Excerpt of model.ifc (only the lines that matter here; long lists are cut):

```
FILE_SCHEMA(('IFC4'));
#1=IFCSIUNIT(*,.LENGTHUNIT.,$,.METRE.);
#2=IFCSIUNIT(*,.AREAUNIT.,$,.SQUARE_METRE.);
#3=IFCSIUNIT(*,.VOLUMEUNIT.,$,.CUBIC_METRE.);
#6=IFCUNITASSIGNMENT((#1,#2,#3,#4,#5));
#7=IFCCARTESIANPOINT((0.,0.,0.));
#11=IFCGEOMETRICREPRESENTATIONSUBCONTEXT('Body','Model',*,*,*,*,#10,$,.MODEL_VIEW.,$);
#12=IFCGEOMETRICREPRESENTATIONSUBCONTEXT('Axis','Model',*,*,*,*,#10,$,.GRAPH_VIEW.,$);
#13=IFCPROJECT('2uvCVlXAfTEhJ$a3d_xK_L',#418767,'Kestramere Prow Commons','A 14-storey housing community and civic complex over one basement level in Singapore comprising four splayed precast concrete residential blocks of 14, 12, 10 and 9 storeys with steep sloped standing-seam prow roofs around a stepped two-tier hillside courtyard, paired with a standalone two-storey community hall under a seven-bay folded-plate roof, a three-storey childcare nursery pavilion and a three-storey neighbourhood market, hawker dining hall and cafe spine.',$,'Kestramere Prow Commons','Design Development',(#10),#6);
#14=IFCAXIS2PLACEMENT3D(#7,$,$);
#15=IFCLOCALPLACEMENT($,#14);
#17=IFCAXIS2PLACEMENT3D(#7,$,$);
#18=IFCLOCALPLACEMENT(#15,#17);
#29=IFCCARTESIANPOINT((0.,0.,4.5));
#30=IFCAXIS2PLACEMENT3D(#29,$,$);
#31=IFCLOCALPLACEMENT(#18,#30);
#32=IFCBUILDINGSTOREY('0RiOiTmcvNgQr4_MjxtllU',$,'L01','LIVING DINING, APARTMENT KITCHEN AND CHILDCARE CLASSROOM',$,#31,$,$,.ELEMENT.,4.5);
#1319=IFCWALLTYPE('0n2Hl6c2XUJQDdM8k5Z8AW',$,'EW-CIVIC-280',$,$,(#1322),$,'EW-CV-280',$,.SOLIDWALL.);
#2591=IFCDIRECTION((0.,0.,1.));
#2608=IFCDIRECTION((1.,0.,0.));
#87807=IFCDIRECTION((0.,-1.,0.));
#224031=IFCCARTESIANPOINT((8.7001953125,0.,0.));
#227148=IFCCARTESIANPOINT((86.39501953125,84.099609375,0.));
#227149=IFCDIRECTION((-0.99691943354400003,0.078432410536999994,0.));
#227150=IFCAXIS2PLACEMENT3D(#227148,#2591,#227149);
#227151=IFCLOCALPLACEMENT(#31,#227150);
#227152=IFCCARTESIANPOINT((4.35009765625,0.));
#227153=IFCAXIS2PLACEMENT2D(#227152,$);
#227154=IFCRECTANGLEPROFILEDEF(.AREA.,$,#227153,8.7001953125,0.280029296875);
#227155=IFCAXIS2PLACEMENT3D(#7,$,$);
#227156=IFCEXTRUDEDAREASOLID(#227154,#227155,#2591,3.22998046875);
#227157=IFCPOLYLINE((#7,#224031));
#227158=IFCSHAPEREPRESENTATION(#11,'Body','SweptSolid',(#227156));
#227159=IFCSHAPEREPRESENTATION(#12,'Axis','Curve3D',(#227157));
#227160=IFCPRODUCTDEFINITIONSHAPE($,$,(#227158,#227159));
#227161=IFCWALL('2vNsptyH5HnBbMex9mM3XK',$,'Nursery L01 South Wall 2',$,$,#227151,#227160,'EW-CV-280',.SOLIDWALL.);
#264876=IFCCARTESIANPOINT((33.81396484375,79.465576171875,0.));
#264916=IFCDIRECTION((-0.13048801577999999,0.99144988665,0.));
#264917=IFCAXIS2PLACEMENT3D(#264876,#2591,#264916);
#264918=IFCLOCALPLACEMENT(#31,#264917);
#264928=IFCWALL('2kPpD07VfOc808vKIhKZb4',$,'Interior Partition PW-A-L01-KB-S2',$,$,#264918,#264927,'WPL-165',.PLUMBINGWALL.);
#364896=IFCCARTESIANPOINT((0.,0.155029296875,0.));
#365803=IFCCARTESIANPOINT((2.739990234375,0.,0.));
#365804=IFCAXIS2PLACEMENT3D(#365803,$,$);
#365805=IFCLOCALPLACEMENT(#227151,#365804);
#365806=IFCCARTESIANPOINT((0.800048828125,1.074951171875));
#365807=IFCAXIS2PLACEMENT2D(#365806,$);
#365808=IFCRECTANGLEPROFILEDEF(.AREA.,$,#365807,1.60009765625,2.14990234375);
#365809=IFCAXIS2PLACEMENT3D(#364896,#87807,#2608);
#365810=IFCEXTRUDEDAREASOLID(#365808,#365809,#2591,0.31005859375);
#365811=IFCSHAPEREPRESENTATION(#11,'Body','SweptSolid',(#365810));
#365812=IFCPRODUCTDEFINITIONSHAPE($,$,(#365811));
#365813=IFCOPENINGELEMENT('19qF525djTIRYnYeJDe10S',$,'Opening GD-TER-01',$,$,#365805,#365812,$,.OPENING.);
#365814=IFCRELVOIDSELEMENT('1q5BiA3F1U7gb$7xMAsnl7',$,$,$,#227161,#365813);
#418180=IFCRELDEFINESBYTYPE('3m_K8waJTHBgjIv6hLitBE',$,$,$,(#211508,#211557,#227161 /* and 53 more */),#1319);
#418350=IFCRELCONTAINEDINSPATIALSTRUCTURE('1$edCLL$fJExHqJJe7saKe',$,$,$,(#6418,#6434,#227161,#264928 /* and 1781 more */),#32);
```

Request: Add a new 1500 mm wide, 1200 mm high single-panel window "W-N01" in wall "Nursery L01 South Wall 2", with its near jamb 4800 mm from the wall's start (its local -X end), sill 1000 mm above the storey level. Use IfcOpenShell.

```python
import numpy as np
import ifcopenshell
import ifcopenshell.api.feature
import ifcopenshell.api.geometry
import ifcopenshell.api.root
import ifcopenshell.api.spatial
import ifcopenshell.geom
import ifcopenshell.util.element
import ifcopenshell.util.placement
import ifcopenshell.util.representation
import ifcopenshell.util.shape
import ifcopenshell.util.unit

model = ifcopenshell.open("model.ifc")
unit_scale = ifcopenshell.util.unit.calculate_unit_scale(model)
settings = ifcopenshell.geom.settings()


def volume(element):
    """Net volume in cubic metres, openings subtracted."""
    shape = ifcopenshell.geom.create_shape(settings, element)
    return ifcopenshell.util.shape.get_volume(shape.geometry)


wall = model.by_id(227161)
storey = ifcopenshell.util.element.get_container(wall, ifc_class="IfcBuildingStorey")
context = ifcopenshell.util.representation.get_context(model, "Model", "Body", "MODEL_VIEW")
before = volume(wall)

width, height, from_end, sill = 1.5, 1.2, 4.8, 1  # metres

# The wall runs along its own X axis, and the end named is its -X end.
wall_shape = ifcopenshell.geom.create_shape(settings, wall)
x, y, z = ifcopenshell.util.shape.get_vertices(wall_shape.geometry).T
start = x.min() + from_end
face, thickness = float(y.min()), float(y.max() - y.min())
wall_matrix = ifcopenshell.util.placement.get_local_placement(wall.ObjectPlacement)
level = ifcopenshell.util.placement.get_local_placement(storey.ObjectPlacement)[2, 3]


def in_wall(x, y):
    """Placement at x, y metres in the wall's axes, at sill height."""
    matrix = wall_matrix.copy()
    matrix[:, 3] = wall_matrix @ np.array([x / unit_scale, y / unit_scale, 0.0, 1.0])
    matrix[2, 3] = level + sill / unit_scale
    return matrix


# Opening: a box that overshoots both wall faces by 50 mm.
opening = ifcopenshell.api.root.create_entity(model, ifc_class="IfcOpeningElement", predefined_type="OPENING")
box = ifcopenshell.api.geometry.add_wall_representation(
    model, context=context, length=width, height=height, thickness=thickness + 0.1
)
ifcopenshell.api.geometry.assign_representation(model, product=opening, representation=box)
ifcopenshell.api.geometry.edit_object_placement(model, product=opening, matrix=in_wall(start, face - 0.05), is_si=False)
ifcopenshell.api.feature.add_feature(model, feature=opening, element=wall)

window = ifcopenshell.api.root.create_entity(model, ifc_class="IfcWindow", name="W-N01", predefined_type="WINDOW")
window.OverallWidth, window.OverallHeight = width / unit_scale, height / unit_scale
window.PartitioningType = "SINGLE_PANEL"
body = ifcopenshell.api.geometry.add_window_representation(
    model,
    context=context,
    overall_width=window.OverallWidth,
    overall_height=window.OverallHeight,
    partition_type="SINGLE_PANEL",
)
ifcopenshell.api.geometry.assign_representation(model, product=window, representation=body)
ifcopenshell.api.spatial.assign_container(model, products=[window], relating_structure=storey)
ifcopenshell.api.feature.add_filling(model, opening=opening, element=window)

# Centre the window in the wall's thickness.
ifcopenshell.api.geometry.edit_object_placement(model, product=window, matrix=in_wall(start, face), is_si=False)
window_shape = ifcopenshell.geom.create_shape(settings, window)
depth = ifcopenshell.util.shape.get_vertices(window_shape.geometry)[:, 1]
offset = face + thickness / 2 - (depth.min() + depth.max()) / 2
ifcopenshell.api.geometry.edit_object_placement(model, product=window, matrix=in_wall(start, offset), is_si=False)

after = volume(wall)

print(f"wall volume {before:.3f} -> {after:.3f} m3")

model.write("model_v2.ifc")
```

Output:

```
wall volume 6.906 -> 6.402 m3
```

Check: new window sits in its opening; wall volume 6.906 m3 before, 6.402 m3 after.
